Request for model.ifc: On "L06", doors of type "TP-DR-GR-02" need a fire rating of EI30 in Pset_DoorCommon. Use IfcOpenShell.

First a look at what the model holds.

```python
import ifcopenshell
import ifcopenshell.util.element

model = ifcopenshell.open("model.ifc")
print(model.schema)
storey = next(s for s in model.by_type("IfcBuildingStorey") if s.Name == "L06")
doors = [e for e in ifcopenshell.util.element.get_decomposition(storey) if e.is_a("IfcDoor")]
seen = {}
for e in doors:
    element_type = ifcopenshell.util.element.get_type(e)
    key = (element_type.Name if element_type != e and element_type else None, ifcopenshell.util.element.get_pset(e, "Pset_DoorCommon", "FireRating"))
    seen[key] = seen.get(key, 0) + 1
for (name, value), count in sorted(seen.items(), key=str):
    print(count, "x", name, "|", value)
```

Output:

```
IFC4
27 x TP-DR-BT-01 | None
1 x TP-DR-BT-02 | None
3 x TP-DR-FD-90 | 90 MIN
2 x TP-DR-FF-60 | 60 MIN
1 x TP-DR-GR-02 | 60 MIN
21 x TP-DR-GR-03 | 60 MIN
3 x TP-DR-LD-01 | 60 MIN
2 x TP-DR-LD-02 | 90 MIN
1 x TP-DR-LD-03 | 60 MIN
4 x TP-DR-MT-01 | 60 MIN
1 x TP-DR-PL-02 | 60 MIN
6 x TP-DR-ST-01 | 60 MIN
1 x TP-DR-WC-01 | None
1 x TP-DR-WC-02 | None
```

```python
import ifcopenshell
import ifcopenshell.api.pset
import ifcopenshell.util.element

model = ifcopenshell.open("model.ifc")

storey = next(s for s in model.by_type("IfcBuildingStorey") if s.Name == "L06")
doors = [e for e in ifcopenshell.util.element.get_decomposition(storey) if e.is_a("IfcDoor")]

count = 0
for e in doors:
    element_type = ifcopenshell.util.element.get_type(e)
    if element_type in (None, e) or element_type.Name != "TP-DR-GR-02":
        continue
    # add_pset returns the element's existing set when there is one.
    pset = ifcopenshell.api.pset.add_pset(model, product=e, name="Pset_DoorCommon")
    ifcopenshell.api.pset.edit_pset(model, pset=pset, properties={"FireRating": "EI30"})
    count += 1

print(count, "doors updated")

model.write("model_rev.ifc")
```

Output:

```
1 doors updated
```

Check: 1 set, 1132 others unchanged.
